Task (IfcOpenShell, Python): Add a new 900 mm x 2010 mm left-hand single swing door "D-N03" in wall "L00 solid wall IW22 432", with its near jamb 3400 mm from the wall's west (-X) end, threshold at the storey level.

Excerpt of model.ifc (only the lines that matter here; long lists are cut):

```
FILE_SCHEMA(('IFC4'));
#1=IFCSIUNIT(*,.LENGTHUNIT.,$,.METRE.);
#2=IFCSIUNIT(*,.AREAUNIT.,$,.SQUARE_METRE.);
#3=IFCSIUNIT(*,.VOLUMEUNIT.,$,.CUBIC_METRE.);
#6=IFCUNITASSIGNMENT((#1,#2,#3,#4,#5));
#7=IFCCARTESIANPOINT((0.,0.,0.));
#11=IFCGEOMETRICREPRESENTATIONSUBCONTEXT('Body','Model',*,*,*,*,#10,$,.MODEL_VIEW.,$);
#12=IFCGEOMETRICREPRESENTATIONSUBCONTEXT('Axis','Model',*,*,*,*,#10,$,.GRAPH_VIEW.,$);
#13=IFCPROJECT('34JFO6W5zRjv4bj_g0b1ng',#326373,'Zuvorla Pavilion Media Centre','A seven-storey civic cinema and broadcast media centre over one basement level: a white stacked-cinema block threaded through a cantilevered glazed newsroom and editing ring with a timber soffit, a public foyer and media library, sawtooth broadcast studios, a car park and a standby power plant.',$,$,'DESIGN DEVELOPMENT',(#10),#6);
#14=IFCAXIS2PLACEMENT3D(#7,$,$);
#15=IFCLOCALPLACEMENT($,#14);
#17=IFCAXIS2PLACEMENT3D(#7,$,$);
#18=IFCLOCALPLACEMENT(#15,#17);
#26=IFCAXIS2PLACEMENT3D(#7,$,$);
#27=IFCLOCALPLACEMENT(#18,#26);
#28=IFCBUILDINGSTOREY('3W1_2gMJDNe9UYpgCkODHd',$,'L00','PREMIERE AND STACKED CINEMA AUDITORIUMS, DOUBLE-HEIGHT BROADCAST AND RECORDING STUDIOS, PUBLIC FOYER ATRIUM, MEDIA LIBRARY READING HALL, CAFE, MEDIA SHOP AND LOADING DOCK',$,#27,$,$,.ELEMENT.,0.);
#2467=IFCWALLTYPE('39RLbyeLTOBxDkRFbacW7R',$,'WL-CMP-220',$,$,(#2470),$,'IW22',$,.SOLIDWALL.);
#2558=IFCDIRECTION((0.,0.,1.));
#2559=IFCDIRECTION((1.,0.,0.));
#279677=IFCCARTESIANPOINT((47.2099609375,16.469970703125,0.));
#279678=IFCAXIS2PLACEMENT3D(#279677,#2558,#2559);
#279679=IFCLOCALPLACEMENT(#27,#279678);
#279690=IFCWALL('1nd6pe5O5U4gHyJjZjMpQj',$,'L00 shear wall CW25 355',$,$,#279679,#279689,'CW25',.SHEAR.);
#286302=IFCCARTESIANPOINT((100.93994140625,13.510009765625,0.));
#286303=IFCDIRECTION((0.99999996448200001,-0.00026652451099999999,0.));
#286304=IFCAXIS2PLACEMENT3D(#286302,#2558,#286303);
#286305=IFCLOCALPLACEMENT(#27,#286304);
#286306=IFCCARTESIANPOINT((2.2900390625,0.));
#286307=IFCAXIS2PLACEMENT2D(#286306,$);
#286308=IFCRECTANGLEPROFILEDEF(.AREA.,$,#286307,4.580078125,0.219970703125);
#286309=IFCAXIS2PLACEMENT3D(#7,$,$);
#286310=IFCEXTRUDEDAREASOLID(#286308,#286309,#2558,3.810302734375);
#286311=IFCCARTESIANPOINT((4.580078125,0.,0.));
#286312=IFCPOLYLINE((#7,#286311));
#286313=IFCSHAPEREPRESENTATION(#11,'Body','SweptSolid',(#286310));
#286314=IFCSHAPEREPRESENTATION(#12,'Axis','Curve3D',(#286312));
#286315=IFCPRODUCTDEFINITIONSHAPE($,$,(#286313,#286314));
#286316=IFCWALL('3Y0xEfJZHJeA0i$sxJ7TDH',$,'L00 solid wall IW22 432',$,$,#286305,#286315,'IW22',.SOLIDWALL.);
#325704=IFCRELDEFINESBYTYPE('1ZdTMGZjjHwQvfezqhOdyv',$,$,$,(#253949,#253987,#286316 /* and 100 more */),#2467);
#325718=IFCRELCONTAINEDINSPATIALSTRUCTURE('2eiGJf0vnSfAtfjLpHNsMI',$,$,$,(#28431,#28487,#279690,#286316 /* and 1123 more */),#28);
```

```python
import numpy as np
import ifcopenshell
import ifcopenshell.api.feature
import ifcopenshell.api.geometry
import ifcopenshell.api.root
import ifcopenshell.api.spatial
import ifcopenshell.geom
import ifcopenshell.util.element
import ifcopenshell.util.placement
import ifcopenshell.util.representation
import ifcopenshell.util.shape
import ifcopenshell.util.unit

model = ifcopenshell.open("model.ifc")
unit_scale = ifcopenshell.util.unit.calculate_unit_scale(model)
settings = ifcopenshell.geom.settings()


def volume(element):
    """Net volume in cubic metres, openings subtracted."""
    shape = ifcopenshell.geom.create_shape(settings, element)
    return ifcopenshell.util.shape.get_volume(shape.geometry)


wall = model.by_guid("3Y0xEfJZHJeA0i$sxJ7TDH")
storey = ifcopenshell.util.element.get_container(wall, ifc_class="IfcBuildingStorey")
context = ifcopenshell.util.representation.get_context(model, "Model", "Body", "MODEL_VIEW")
before = volume(wall)

width, height, from_end, sill = 0.9, 2.01, 3.4, 0.0  # metres

# The wall runs along its own X axis, and the end named is its -X end.
wall_shape = ifcopenshell.geom.create_shape(settings, wall)
x, y, z = ifcopenshell.util.shape.get_vertices(wall_shape.geometry).T
start = x.min() + from_end
face, thickness = float(y.min()), float(y.max() - y.min())
wall_matrix = ifcopenshell.util.placement.get_local_placement(wall.ObjectPlacement)
level = ifcopenshell.util.placement.get_local_placement(storey.ObjectPlacement)[2, 3]


def in_wall(x, y):
    """Placement at x, y metres in the wall's axes, at sill height."""
    matrix = wall_matrix.copy()
    matrix[:, 3] = wall_matrix @ np.array([x / unit_scale, y / unit_scale, 0.0, 1.0])
    matrix[2, 3] = level + sill / unit_scale
    return matrix


# Opening: a box that overshoots both wall faces by 50 mm.
opening = ifcopenshell.api.root.create_entity(model, ifc_class="IfcOpeningElement", predefined_type="OPENING")
box = ifcopenshell.api.geometry.add_wall_representation(
    model, context=context, length=width, height=height, thickness=thickness + 0.1
)
ifcopenshell.api.geometry.assign_representation(model, product=opening, representation=box)
ifcopenshell.api.geometry.edit_object_placement(model, product=opening, matrix=in_wall(start, face - 0.05), is_si=False)
ifcopenshell.api.feature.add_feature(model, feature=opening, element=wall)

door = ifcopenshell.api.root.create_entity(model, ifc_class="IfcDoor", name="D-N03", predefined_type="DOOR")
door.OverallWidth, door.OverallHeight = width / unit_scale, height / unit_scale
door.OperationType = "SINGLE_SWING_LEFT"
body = ifcopenshell.api.geometry.add_door_representation(
    model,
    context=context,
    overall_width=door.OverallWidth,
    overall_height=door.OverallHeight,
    operation_type="SINGLE_SWING_LEFT",
    lining_properties={"LiningDepth": thickness / unit_scale, "ThresholdDepth": thickness / unit_scale},
)
ifcopenshell.api.geometry.assign_representation(model, product=door, representation=body)
ifcopenshell.api.spatial.assign_container(model, products=[door], relating_structure=storey)
ifcopenshell.api.feature.add_filling(model, opening=opening, element=door)

# The lining spans the wall, so the door starts at the wall face.
ifcopenshell.api.geometry.edit_object_placement(model, product=door, matrix=in_wall(start, face), is_si=False)

after = volume(wall)

print(f"wall volume {before:.3f} -> {after:.3f} m3")

model.write("model_edited.ifc")
```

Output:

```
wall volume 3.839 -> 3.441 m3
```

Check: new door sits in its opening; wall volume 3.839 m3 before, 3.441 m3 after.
